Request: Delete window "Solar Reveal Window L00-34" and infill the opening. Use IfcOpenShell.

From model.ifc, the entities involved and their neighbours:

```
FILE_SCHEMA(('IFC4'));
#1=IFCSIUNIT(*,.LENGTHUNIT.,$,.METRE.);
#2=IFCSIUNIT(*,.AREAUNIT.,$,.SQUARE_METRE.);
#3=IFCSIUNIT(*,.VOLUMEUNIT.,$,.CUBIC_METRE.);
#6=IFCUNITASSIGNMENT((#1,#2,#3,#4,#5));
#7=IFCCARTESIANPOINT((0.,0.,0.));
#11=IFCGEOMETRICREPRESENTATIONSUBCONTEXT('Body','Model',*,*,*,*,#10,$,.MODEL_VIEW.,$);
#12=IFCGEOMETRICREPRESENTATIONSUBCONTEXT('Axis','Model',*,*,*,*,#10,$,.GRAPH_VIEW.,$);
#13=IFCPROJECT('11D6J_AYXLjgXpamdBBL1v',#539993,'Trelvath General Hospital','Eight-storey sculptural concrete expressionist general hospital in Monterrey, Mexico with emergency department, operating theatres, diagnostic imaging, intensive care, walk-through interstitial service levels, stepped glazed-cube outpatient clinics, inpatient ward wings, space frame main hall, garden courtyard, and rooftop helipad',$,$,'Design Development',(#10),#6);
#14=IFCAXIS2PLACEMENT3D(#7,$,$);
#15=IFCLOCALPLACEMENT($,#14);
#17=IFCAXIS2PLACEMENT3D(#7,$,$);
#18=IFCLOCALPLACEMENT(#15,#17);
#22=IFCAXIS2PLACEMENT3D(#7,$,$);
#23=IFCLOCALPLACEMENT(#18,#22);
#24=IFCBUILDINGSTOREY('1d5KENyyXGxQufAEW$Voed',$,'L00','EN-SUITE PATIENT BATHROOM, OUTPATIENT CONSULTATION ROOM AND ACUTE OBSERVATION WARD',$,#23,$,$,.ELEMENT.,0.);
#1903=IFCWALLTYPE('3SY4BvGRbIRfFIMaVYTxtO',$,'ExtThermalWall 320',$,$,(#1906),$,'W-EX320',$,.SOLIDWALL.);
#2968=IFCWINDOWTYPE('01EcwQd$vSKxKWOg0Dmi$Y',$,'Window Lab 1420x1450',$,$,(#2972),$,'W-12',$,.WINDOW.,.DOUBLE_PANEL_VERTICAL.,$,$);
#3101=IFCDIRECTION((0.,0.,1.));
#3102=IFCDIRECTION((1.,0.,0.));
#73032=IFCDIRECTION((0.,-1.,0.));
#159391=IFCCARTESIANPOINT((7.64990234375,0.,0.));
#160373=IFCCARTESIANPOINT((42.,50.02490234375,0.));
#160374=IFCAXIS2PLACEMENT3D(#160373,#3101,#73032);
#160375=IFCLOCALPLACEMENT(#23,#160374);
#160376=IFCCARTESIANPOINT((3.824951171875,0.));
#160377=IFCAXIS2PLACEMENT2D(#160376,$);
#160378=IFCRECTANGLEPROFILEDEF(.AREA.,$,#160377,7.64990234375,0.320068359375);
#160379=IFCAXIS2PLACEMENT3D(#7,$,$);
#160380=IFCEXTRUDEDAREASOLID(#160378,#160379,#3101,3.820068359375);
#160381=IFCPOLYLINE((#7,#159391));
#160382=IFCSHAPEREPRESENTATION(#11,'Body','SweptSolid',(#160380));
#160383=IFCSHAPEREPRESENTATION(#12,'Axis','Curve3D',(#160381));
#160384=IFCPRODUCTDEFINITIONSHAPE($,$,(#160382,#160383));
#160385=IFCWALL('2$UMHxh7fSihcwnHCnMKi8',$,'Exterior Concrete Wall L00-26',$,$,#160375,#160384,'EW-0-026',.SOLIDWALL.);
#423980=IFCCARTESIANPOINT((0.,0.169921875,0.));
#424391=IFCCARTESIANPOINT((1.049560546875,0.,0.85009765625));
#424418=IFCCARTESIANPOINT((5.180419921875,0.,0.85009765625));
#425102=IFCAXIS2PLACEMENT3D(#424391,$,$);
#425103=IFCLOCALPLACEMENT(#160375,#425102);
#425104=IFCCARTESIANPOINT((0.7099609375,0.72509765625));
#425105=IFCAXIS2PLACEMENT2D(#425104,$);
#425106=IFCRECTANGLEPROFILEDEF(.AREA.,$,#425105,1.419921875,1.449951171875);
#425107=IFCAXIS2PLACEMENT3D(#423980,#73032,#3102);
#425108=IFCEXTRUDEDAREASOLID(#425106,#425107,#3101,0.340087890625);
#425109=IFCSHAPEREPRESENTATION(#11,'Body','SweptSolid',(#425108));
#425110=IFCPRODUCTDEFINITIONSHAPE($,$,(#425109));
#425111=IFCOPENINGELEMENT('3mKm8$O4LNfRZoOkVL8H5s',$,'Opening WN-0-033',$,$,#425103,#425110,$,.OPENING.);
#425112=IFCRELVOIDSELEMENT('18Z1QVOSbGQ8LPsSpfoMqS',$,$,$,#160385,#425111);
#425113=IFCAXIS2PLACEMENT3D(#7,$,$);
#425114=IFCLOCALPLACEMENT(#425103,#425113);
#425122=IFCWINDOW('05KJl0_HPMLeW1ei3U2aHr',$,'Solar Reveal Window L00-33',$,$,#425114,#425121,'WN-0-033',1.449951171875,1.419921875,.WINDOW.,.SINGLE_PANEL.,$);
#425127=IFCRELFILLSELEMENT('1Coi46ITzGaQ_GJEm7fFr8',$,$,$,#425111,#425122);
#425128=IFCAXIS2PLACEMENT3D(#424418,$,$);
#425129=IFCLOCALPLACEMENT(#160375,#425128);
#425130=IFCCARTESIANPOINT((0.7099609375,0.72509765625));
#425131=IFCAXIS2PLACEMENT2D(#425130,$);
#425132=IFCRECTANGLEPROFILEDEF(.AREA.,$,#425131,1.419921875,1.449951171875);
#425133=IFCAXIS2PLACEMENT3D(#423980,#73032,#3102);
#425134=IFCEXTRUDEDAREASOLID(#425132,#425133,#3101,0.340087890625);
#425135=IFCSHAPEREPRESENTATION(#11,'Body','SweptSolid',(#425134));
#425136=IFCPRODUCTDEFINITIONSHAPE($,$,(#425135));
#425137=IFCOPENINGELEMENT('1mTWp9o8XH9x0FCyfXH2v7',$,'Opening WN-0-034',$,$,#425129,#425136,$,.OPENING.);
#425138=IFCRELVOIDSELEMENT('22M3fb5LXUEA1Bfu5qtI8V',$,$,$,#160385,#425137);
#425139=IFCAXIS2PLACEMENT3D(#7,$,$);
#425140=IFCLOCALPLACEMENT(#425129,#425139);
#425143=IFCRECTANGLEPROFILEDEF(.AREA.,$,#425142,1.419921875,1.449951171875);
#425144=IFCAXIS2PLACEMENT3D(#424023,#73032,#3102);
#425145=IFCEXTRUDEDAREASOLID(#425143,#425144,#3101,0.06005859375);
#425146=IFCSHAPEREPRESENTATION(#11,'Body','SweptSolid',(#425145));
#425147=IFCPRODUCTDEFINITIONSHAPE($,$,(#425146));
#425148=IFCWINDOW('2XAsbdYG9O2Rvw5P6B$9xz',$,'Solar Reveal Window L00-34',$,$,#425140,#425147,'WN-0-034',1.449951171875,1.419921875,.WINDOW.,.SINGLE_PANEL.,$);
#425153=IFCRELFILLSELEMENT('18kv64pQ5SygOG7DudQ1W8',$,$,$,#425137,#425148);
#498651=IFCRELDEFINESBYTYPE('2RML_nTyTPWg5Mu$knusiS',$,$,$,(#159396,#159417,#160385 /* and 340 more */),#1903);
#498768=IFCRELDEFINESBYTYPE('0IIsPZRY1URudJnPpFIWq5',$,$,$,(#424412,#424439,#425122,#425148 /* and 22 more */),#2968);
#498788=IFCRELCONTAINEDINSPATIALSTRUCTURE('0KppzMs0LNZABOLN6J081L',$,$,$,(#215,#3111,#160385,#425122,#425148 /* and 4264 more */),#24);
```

```python
import ifcopenshell
import ifcopenshell.api.feature
import ifcopenshell.api.root
import ifcopenshell.geom
import ifcopenshell.util.shape

model = ifcopenshell.open("model.ifc")
settings = ifcopenshell.geom.settings()


def volume(element):
    """Net volume in cubic metres, openings subtracted."""
    shape = ifcopenshell.geom.create_shape(settings, element)
    return ifcopenshell.util.shape.get_volume(shape.geometry)


window = model.by_guid("2XAsbdYG9O2Rvw5P6B$9xz")
opening = window.FillsVoids[0].RelatingOpeningElement
wall = opening.VoidsElements[0].RelatingBuildingElement
before = volume(wall)

ifcopenshell.api.root.remove_product(model, product=window)
ifcopenshell.api.feature.remove_feature(model, feature=opening)

after = volume(wall)

print(f"wall volume {before:.3f} -> {after:.3f} m3")

model.write("model_updated.ifc")
```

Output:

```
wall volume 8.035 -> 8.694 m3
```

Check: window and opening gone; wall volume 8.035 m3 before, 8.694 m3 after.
